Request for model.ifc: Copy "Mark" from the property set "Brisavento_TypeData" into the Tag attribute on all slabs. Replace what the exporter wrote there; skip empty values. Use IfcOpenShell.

First a look at what the model holds.

```python
import ifcopenshell
import ifcopenshell.util.element

model = ifcopenshell.open("model.ifc")
print(model.schema)
slabs = model.by_type("IfcSlab")
print(len(slabs), "slabs")
for e in slabs[:8]:
    source = ifcopenshell.util.element.get_pset(e, "Brisavento_TypeData", "Mark")
    target = e.Tag
    print(e.id(), repr(source), repr(target), sep=" | ")
```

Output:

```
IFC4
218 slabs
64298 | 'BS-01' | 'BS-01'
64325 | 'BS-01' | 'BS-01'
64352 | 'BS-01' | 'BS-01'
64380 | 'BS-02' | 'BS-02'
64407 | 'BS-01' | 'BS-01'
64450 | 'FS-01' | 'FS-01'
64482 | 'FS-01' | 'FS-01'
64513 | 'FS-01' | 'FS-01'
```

```python
import ifcopenshell
import ifcopenshell.util.element

model = ifcopenshell.open("model.ifc")

count = 0
for e in model.by_type("IfcSlab"):
    value = ifcopenshell.util.element.get_pset(e, "Brisavento_TypeData", "Mark")
    current = e.Tag
    if not value or not value.strip() or current == value:
        continue
    e.Tag = value
    count += 1

print(count, "slabs updated")

model.write("model_rev.ifc")
```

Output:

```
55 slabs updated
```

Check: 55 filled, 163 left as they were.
